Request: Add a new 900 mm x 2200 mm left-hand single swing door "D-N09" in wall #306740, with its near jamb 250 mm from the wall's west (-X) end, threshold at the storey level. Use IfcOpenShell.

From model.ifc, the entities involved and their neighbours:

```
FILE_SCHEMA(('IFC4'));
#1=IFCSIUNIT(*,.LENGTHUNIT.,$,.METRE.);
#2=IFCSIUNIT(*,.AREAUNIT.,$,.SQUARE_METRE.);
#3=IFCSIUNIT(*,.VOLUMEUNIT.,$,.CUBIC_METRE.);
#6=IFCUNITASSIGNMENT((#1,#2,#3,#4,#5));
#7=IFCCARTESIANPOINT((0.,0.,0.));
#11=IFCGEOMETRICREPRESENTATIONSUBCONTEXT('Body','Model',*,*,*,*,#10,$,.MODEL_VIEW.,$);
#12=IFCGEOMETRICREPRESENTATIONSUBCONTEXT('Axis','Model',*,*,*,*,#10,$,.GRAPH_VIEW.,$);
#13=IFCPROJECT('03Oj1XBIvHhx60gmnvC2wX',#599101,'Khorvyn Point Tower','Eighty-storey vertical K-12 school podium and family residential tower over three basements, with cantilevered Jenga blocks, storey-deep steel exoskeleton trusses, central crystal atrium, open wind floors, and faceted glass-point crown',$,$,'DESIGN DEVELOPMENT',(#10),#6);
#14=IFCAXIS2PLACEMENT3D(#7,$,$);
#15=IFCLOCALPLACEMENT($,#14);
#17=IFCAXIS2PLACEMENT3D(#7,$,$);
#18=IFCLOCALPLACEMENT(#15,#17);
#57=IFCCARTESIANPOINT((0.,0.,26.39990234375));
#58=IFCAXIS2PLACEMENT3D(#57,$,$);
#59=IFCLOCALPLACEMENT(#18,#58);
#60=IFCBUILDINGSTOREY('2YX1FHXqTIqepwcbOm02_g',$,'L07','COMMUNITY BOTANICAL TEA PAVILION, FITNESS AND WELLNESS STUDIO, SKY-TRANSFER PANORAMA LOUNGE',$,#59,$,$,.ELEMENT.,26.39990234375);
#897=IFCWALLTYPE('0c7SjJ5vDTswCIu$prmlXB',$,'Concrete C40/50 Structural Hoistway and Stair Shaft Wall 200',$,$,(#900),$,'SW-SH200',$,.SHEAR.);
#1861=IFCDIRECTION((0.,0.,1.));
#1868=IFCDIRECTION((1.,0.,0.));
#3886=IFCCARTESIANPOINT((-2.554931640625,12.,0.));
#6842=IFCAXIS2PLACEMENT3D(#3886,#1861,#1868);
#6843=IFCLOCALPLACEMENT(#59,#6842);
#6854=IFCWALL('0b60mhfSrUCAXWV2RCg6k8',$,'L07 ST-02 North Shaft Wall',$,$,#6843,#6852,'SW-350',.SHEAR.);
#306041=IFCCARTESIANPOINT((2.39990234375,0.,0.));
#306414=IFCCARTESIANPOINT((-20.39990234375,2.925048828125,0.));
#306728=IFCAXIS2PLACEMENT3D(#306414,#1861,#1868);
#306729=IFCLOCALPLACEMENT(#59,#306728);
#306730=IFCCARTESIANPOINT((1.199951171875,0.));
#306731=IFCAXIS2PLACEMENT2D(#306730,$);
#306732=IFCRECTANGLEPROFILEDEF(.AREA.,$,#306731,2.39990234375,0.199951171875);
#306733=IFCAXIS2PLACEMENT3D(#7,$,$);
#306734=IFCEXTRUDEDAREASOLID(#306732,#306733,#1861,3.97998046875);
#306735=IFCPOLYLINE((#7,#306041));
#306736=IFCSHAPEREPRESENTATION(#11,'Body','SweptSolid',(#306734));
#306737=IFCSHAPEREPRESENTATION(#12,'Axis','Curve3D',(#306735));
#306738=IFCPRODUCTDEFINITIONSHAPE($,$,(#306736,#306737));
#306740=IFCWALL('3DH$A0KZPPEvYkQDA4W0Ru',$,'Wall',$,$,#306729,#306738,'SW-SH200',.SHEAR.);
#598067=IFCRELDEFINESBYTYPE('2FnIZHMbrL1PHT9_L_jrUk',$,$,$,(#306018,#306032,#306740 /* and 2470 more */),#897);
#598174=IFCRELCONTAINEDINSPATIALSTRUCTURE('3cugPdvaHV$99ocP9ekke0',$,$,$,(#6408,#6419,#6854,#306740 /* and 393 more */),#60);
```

```python
import numpy as np
import ifcopenshell
import ifcopenshell.api.feature
import ifcopenshell.api.geometry
import ifcopenshell.api.root
import ifcopenshell.api.spatial
import ifcopenshell.geom
import ifcopenshell.util.element
import ifcopenshell.util.placement
import ifcopenshell.util.representation
import ifcopenshell.util.shape
import ifcopenshell.util.unit

model = ifcopenshell.open("model.ifc")
unit_scale = ifcopenshell.util.unit.calculate_unit_scale(model)
settings = ifcopenshell.geom.settings()


def volume(element):
    """Net volume in cubic metres, openings subtracted."""
    shape = ifcopenshell.geom.create_shape(settings, element)
    return ifcopenshell.util.shape.get_volume(shape.geometry)


wall = model.by_guid("3DH$A0KZPPEvYkQDA4W0Ru")
storey = ifcopenshell.util.element.get_container(wall, ifc_class="IfcBuildingStorey")
context = ifcopenshell.util.representation.get_context(model, "Model", "Body", "MODEL_VIEW")
before = volume(wall)

width, height, from_end, sill = 0.9, 2.2, 0.25, 0.0  # metres

# The wall runs along its own X axis, and the end named is its -X end.
wall_shape = ifcopenshell.geom.create_shape(settings, wall)
x, y, z = ifcopenshell.util.shape.get_vertices(wall_shape.geometry).T
start = x.min() + from_end
face, thickness = float(y.min()), float(y.max() - y.min())
wall_matrix = ifcopenshell.util.placement.get_local_placement(wall.ObjectPlacement)
level = ifcopenshell.util.placement.get_local_placement(storey.ObjectPlacement)[2, 3]


def in_wall(x, y):
    """Placement at x, y metres in the wall's axes, at sill height."""
    matrix = wall_matrix.copy()
    matrix[:, 3] = wall_matrix @ np.array([x / unit_scale, y / unit_scale, 0.0, 1.0])
    matrix[2, 3] = level + sill / unit_scale
    return matrix


# Opening: a box that overshoots both wall faces by 50 mm.
opening = ifcopenshell.api.root.create_entity(model, ifc_class="IfcOpeningElement", predefined_type="OPENING")
box = ifcopenshell.api.geometry.add_wall_representation(
    model, context=context, length=width, height=height, thickness=thickness + 0.1
)
ifcopenshell.api.geometry.assign_representation(model, product=opening, representation=box)
ifcopenshell.api.geometry.edit_object_placement(model, product=opening, matrix=in_wall(start, face - 0.05), is_si=False)
ifcopenshell.api.feature.add_feature(model, feature=opening, element=wall)

door = ifcopenshell.api.root.create_entity(model, ifc_class="IfcDoor", name="D-N09", predefined_type="DOOR")
door.OverallWidth, door.OverallHeight = width / unit_scale, height / unit_scale
door.OperationType = "SINGLE_SWING_LEFT"
body = ifcopenshell.api.geometry.add_door_representation(
    model,
    context=context,
    overall_width=door.OverallWidth,
    overall_height=door.OverallHeight,
    operation_type="SINGLE_SWING_LEFT",
    lining_properties={"LiningDepth": thickness / unit_scale, "ThresholdDepth": thickness / unit_scale},
)
ifcopenshell.api.geometry.assign_representation(model, product=door, representation=body)
ifcopenshell.api.spatial.assign_container(model, products=[door], relating_structure=storey)
ifcopenshell.api.feature.add_filling(model, opening=opening, element=door)

# The lining spans the wall, so the door starts at the wall face.
ifcopenshell.api.geometry.edit_object_placement(model, product=door, matrix=in_wall(start, face), is_si=False)

after = volume(wall)

print(f"wall volume {before:.3f} -> {after:.3f} m3")

model.write("model_v2.ifc")
```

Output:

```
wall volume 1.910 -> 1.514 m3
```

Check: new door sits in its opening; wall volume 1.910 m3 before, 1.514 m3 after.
